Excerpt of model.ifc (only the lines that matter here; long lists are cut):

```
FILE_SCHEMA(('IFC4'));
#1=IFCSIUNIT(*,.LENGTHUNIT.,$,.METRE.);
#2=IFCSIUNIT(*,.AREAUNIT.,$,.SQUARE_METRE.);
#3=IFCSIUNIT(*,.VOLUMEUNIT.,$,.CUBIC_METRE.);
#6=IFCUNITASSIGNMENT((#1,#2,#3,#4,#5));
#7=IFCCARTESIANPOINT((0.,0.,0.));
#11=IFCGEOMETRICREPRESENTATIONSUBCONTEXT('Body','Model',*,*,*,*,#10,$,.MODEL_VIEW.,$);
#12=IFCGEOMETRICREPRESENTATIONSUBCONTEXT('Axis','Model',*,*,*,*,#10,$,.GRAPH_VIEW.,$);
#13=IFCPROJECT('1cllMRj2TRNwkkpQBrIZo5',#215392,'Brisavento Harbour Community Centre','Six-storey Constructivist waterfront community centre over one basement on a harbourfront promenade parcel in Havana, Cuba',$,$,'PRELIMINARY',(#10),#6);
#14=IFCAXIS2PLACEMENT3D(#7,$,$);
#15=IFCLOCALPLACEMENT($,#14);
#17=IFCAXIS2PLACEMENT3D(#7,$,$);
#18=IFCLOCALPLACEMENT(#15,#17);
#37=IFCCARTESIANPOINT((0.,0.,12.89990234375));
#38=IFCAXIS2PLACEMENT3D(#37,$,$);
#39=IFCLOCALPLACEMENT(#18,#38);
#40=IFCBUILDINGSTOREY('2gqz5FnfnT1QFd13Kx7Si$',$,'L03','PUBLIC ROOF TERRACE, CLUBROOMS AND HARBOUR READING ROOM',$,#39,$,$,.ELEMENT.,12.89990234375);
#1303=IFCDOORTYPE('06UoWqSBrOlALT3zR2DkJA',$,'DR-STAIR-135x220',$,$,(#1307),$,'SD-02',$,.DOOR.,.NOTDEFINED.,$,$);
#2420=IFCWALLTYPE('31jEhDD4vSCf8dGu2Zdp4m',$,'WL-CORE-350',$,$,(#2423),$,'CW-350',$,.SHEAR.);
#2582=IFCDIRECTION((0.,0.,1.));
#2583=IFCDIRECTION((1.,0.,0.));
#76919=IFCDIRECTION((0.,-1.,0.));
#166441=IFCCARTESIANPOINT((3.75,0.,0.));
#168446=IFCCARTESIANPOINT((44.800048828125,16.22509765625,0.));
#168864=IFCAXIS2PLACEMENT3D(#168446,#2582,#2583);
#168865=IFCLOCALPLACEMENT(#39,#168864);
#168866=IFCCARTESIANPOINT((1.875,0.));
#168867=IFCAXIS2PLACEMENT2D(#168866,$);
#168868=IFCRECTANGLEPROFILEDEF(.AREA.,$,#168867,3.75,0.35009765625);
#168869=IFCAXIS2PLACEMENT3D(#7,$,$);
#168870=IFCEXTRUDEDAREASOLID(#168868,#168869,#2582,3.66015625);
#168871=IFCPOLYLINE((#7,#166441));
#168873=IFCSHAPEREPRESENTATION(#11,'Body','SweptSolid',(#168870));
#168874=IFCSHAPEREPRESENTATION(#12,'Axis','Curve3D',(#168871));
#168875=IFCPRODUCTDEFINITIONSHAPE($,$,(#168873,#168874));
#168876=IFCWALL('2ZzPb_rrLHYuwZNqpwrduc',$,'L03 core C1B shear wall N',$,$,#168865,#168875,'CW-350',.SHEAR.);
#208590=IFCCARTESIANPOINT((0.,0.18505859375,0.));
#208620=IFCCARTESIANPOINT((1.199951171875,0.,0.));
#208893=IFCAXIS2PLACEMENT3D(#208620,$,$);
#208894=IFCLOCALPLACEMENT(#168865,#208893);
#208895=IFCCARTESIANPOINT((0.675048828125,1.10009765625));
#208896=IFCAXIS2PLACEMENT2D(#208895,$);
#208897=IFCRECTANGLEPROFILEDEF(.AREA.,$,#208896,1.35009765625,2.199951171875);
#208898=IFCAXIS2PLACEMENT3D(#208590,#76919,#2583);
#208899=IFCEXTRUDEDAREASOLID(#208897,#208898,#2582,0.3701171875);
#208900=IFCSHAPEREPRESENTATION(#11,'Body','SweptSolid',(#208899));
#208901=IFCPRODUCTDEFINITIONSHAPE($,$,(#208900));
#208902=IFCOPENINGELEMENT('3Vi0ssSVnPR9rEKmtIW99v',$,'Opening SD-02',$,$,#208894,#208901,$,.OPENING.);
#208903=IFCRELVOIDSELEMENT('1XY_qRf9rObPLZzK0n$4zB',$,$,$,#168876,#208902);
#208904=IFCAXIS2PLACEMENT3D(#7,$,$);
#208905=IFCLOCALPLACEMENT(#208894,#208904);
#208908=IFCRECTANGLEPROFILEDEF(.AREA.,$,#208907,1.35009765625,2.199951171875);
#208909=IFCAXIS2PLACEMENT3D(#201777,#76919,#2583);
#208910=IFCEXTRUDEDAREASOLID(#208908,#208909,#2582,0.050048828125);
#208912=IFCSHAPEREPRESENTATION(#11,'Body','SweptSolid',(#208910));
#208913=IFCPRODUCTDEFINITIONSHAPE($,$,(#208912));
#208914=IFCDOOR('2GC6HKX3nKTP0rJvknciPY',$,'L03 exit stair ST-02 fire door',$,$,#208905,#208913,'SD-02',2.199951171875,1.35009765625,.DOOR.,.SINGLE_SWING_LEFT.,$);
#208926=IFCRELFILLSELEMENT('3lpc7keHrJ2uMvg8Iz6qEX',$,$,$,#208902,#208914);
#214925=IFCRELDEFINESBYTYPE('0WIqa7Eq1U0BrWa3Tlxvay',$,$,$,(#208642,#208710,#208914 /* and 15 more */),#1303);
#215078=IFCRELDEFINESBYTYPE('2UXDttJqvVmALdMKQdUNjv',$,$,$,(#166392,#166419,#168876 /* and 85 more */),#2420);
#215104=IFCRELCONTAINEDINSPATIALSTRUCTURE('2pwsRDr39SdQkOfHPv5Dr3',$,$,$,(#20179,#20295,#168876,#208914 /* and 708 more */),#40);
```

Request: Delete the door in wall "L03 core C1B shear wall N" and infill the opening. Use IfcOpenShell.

```python
import ifcopenshell
import ifcopenshell.api.feature
import ifcopenshell.api.root
import ifcopenshell.geom
import ifcopenshell.util.shape

model = ifcopenshell.open("model.ifc")
settings = ifcopenshell.geom.settings()


def volume(element):
    """Net volume in cubic metres, openings subtracted."""
    shape = ifcopenshell.geom.create_shape(settings, element)
    return ifcopenshell.util.shape.get_volume(shape.geometry)


door = model.by_guid("2GC6HKX3nKTP0rJvknciPY")
opening = door.FillsVoids[0].RelatingOpeningElement
wall = opening.VoidsElements[0].RelatingBuildingElement
before = volume(wall)

ifcopenshell.api.root.remove_product(model, product=door)
ifcopenshell.api.feature.remove_feature(model, feature=opening)

after = volume(wall)

print(f"wall volume {before:.3f} -> {after:.3f} m3")

model.write("model_edited.ifc")
```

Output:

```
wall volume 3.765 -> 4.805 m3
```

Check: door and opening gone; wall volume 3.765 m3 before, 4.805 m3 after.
